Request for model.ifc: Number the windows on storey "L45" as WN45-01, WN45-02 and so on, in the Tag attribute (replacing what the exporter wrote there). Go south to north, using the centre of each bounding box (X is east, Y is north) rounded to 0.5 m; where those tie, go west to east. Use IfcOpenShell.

First a look at what the model holds.

```python
import ifcopenshell
import ifcopenshell.util.element
import ifcopenshell.util.placement

model = ifcopenshell.open("model.ifc")
print(model.schema)
storey = next(s for s in model.by_type("IfcBuildingStorey") if s.Name == "L45")
windows = [e for e in ifcopenshell.util.element.get_decomposition(storey) if e.is_a("IfcWindow")]
for e in sorted(windows, key=lambda e: e.id()):
    origin = ifcopenshell.util.placement.get_local_placement(e.ObjectPlacement)[:3, 3]
    print(e.id(), e.Tag, e.Name, origin.round(2) + 0.0, sep=" | ")
```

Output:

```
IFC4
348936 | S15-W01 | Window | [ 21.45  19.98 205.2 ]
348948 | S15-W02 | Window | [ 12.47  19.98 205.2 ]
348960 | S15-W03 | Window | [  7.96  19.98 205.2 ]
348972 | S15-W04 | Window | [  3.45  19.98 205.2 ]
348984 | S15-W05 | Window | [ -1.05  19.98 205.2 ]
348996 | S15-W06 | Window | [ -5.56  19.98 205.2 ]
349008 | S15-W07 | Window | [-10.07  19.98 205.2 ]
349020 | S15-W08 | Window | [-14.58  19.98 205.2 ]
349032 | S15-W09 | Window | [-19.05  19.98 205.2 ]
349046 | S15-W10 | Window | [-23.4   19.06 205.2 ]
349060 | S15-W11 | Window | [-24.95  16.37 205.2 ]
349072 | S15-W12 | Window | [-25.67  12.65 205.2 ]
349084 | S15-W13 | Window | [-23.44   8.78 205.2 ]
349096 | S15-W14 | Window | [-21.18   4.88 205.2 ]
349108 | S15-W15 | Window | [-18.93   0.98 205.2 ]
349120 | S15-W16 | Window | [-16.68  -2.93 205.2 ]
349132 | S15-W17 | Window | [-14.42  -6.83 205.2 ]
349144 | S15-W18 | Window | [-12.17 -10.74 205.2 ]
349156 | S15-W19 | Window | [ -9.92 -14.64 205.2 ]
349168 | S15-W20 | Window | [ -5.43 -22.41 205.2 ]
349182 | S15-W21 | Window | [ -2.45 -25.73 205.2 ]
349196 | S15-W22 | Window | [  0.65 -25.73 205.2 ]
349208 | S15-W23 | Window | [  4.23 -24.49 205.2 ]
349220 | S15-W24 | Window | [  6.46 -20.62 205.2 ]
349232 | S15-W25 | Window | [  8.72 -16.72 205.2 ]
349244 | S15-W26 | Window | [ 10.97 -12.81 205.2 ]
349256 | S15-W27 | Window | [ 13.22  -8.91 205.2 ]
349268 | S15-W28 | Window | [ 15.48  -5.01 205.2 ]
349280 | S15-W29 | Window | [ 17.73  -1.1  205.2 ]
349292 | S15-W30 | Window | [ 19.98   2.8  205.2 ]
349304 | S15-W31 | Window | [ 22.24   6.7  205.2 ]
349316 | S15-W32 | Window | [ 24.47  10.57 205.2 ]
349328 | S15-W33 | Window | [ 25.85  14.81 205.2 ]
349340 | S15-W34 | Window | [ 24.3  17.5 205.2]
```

```python
import ifcopenshell
import ifcopenshell.geom
import ifcopenshell.util.element
import ifcopenshell.util.shape

model = ifcopenshell.open("model.ifc")
settings = ifcopenshell.geom.settings()
settings.set("use-world-coords", True)


def centre(element):
    shape = ifcopenshell.geom.create_shape(settings, element)
    return ifcopenshell.util.shape.get_bbox_centroid(shape.geometry)


storey = next(s for s in model.by_type("IfcBuildingStorey") if s.Name == "L45")
windows = [e for e in ifcopenshell.util.element.get_decomposition(storey) if e.is_a("IfcWindow")]

# Insertion points can sit at a corner or the storey origin, so sort by the geometry (in metres).
centres = {e: centre(e) for e in windows}
windows.sort(key=lambda e: (round(centres[e][1] / 0.5), centres[e][0]))

for i, e in enumerate(windows, start=1):
    number = f"WN45-{i:02d}"
    e.Tag = number
    print(e.id(), number)

model.write("model_rev.ifc")
```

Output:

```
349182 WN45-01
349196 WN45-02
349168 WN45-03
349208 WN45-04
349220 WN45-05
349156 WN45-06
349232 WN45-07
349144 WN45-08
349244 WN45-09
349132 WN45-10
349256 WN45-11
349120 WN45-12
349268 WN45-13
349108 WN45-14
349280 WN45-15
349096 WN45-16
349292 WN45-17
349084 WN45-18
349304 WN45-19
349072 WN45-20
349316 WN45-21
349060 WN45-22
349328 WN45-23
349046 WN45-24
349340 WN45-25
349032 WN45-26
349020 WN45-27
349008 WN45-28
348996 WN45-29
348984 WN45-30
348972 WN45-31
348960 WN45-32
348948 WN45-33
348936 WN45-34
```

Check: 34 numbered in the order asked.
